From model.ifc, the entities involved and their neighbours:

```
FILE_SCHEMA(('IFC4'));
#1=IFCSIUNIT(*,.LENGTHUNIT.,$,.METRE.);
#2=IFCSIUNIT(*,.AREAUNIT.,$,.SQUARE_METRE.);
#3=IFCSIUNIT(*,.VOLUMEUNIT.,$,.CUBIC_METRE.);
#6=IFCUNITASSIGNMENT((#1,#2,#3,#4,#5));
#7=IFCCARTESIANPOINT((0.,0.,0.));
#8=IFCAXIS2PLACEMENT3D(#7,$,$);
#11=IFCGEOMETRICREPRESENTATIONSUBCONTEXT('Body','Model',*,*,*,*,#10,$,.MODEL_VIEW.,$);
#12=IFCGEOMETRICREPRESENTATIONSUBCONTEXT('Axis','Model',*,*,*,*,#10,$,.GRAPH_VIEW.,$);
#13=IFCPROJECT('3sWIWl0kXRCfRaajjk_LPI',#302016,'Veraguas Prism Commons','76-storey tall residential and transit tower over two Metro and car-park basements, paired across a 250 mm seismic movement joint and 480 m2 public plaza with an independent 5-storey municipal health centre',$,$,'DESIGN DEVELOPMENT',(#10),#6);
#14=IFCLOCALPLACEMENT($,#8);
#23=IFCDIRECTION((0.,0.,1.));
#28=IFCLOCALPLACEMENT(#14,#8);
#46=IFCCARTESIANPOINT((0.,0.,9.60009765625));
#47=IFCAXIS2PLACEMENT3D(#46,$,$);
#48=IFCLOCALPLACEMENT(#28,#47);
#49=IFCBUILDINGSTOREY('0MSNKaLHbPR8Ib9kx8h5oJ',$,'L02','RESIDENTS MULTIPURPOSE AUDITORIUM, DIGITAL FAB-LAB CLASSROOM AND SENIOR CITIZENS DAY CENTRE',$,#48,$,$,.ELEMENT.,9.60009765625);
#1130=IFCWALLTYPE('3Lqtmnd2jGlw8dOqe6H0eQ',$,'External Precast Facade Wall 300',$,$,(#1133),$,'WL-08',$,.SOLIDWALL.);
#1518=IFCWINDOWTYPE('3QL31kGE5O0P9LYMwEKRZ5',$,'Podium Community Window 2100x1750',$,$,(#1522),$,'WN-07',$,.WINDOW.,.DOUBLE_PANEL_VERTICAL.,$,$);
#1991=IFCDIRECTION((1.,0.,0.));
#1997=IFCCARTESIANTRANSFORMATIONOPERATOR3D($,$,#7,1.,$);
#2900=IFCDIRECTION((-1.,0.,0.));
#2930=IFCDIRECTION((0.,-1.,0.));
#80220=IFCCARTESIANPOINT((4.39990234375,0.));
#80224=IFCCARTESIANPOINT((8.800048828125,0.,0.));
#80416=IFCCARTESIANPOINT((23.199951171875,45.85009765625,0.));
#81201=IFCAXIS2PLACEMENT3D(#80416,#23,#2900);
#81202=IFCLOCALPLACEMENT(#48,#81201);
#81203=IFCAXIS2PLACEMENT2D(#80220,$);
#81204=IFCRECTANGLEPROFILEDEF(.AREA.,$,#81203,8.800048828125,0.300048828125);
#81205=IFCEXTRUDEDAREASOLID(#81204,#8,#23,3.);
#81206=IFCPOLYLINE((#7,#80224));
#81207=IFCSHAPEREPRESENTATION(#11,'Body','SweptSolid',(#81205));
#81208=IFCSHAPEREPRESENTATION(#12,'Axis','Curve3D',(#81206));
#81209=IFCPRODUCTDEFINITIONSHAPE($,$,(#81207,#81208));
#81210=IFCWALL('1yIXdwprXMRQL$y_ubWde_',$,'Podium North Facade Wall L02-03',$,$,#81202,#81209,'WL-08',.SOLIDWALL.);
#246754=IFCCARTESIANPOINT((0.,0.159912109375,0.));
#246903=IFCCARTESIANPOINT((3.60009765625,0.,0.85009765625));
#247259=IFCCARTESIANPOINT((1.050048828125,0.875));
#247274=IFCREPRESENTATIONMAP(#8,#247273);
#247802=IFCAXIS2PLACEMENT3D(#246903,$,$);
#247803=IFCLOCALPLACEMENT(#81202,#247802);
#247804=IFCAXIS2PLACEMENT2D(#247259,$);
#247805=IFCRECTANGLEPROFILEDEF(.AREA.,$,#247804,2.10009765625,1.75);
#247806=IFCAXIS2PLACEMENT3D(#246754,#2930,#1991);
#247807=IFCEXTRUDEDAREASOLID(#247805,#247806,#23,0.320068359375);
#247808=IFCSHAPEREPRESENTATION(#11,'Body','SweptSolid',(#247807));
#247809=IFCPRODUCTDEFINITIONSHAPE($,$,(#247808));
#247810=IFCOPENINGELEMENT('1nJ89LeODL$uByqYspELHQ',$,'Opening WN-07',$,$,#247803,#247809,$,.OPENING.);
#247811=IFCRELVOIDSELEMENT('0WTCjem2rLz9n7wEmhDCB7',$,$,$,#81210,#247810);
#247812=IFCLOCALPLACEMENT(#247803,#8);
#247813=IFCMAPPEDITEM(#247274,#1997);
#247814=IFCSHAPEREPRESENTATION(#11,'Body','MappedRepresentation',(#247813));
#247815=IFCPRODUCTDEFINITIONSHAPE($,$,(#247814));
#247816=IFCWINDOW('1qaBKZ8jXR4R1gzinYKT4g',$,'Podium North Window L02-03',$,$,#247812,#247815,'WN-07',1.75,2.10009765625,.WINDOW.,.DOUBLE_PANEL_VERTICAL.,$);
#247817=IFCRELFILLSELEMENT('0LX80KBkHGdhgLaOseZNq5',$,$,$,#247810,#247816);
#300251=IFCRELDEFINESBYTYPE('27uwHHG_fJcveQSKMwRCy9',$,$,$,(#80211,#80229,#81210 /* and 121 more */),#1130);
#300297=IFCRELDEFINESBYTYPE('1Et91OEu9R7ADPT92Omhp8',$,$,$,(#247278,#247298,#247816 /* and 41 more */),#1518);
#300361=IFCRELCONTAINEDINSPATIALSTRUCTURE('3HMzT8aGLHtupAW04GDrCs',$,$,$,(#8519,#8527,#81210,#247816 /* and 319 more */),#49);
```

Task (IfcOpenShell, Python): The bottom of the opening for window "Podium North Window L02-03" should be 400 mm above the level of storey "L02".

```python
import numpy as np
import ifcopenshell
import ifcopenshell.api.geometry
import ifcopenshell.geom
import ifcopenshell.util.element
import ifcopenshell.util.placement
import ifcopenshell.util.shape
import ifcopenshell.util.unit

model = ifcopenshell.open("model.ifc")
unit_scale = ifcopenshell.util.unit.calculate_unit_scale(model)

window = model.by_id(247816)
opening = window.FillsVoids[0].RelatingOpeningElement
storey = ifcopenshell.util.element.get_container(window, ifc_class="IfcBuildingStorey")
level = ifcopenshell.util.placement.get_local_placement(storey.ObjectPlacement)[2, 3]

# The opening's origin need not be at the sill, so measure its lowest point.
shape = ifcopenshell.geom.create_shape(ifcopenshell.geom.settings(), opening)
bottom = ifcopenshell.util.shape.get_shape_bottom_elevation(shape, shape.geometry) / unit_scale
dz = level + 0.4 - bottom

shift = np.array([0.0, 0.0, dz])
# The window is placed relative to its opening, so it follows when the opening moves.
matrix = ifcopenshell.util.placement.get_local_placement(opening.ObjectPlacement)
matrix[:3, 3] += shift
ifcopenshell.api.geometry.edit_object_placement(
    model, product=opening, matrix=matrix, is_si=False, should_transform_children=True
)

print(f"moved by {dz * unit_scale:+.3f} m")

model.write("model_rev.ifc")
```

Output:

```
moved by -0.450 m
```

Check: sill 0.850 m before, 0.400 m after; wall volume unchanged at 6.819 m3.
